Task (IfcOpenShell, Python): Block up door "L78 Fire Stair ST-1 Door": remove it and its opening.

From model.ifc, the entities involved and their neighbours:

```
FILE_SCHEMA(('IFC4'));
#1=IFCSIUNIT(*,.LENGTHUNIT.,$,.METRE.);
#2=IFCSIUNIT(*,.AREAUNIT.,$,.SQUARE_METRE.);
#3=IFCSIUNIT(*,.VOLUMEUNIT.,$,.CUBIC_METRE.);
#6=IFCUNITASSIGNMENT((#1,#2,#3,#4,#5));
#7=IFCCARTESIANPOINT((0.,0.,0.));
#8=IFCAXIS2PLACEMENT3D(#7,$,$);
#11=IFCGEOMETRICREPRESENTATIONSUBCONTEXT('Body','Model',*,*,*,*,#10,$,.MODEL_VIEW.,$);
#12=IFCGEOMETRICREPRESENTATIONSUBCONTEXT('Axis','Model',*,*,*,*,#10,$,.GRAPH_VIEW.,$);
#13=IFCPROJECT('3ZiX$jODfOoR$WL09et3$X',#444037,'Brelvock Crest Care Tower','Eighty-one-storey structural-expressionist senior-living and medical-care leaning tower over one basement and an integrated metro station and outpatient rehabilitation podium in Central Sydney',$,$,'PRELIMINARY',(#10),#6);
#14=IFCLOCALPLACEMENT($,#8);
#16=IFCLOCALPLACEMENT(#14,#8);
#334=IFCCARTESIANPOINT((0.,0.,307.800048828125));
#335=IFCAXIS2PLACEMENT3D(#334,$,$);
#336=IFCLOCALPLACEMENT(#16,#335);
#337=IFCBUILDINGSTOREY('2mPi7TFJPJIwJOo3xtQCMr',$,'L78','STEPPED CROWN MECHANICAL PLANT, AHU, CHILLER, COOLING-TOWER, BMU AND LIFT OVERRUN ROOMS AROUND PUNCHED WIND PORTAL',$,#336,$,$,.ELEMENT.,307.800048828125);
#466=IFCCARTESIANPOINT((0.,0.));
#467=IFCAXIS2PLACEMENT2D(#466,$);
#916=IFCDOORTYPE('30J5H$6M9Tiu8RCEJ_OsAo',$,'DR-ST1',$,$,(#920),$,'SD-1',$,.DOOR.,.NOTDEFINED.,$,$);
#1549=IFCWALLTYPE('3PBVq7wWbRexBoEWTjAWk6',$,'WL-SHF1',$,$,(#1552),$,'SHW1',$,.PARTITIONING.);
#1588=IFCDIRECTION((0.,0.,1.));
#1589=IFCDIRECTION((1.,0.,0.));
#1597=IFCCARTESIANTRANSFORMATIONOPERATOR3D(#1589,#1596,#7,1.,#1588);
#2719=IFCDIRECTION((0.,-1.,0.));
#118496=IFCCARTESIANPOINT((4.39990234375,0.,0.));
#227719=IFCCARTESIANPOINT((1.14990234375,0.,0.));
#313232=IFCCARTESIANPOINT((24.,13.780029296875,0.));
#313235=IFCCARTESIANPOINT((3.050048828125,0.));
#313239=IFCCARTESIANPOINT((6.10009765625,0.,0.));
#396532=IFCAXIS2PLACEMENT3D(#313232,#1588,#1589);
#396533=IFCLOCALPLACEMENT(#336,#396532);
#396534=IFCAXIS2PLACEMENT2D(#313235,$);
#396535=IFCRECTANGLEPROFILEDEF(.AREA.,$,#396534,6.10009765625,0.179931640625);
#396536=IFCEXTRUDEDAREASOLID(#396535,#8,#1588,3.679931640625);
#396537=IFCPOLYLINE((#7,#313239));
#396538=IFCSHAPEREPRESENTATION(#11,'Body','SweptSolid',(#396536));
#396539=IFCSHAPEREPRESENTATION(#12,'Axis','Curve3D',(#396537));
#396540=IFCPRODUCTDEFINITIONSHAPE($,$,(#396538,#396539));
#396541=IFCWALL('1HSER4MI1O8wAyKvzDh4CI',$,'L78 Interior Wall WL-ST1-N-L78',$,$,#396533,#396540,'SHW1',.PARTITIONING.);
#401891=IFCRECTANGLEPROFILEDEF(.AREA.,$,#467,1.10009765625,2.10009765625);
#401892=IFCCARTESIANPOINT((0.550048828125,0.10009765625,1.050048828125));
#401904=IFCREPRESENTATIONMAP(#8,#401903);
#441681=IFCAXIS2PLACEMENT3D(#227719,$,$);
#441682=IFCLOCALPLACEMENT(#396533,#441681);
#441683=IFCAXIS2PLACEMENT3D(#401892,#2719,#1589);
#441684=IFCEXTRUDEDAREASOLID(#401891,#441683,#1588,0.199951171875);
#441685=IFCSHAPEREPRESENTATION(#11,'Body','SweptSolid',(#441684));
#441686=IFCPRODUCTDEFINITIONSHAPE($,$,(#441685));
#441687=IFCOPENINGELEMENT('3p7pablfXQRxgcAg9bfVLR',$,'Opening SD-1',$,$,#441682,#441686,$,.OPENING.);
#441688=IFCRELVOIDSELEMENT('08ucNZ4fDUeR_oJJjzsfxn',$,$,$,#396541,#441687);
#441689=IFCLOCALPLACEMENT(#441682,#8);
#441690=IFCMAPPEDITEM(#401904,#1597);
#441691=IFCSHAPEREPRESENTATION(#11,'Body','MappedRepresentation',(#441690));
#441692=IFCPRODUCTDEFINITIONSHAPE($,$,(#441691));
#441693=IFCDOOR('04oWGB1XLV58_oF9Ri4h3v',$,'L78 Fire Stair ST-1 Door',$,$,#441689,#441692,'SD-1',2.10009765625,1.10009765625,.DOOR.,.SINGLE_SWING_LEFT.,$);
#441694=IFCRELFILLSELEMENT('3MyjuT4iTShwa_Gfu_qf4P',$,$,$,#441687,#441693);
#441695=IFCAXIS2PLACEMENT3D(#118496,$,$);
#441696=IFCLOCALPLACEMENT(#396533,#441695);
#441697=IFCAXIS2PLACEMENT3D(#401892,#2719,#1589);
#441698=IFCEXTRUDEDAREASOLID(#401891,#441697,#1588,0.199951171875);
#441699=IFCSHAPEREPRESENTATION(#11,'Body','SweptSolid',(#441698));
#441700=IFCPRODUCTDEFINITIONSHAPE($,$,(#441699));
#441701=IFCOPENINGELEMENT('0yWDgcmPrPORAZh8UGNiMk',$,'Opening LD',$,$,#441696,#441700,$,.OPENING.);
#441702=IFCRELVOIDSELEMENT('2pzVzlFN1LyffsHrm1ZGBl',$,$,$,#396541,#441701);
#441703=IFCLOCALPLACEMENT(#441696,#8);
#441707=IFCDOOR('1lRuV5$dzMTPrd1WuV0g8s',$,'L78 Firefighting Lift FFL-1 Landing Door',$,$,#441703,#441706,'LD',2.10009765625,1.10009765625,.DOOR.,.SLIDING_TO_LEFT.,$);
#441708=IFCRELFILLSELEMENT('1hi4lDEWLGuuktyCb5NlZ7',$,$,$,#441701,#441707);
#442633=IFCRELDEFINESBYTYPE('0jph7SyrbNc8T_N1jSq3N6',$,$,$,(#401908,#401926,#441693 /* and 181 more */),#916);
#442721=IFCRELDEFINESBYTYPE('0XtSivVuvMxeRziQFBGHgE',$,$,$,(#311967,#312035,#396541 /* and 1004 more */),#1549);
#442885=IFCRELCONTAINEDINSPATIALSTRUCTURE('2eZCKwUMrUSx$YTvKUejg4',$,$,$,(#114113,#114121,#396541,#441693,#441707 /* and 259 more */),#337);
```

```python
import ifcopenshell
import ifcopenshell.api.feature
import ifcopenshell.api.root
import ifcopenshell.geom
import ifcopenshell.util.shape

model = ifcopenshell.open("model.ifc")
settings = ifcopenshell.geom.settings()


def volume(element):
    """Net volume in cubic metres, openings subtracted."""
    shape = ifcopenshell.geom.create_shape(settings, element)
    return ifcopenshell.util.shape.get_volume(shape.geometry)


door = model.by_guid("04oWGB1XLV58_oF9Ri4h3v")
opening = door.FillsVoids[0].RelatingOpeningElement
wall = opening.VoidsElements[0].RelatingBuildingElement
before = volume(wall)

ifcopenshell.api.root.remove_product(model, product=door)
ifcopenshell.api.feature.remove_feature(model, feature=opening)

after = volume(wall)

print(f"wall volume {before:.3f} -> {after:.3f} m3")

model.write("model_edited.ifc")
```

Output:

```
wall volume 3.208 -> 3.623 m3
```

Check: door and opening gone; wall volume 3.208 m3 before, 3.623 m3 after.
